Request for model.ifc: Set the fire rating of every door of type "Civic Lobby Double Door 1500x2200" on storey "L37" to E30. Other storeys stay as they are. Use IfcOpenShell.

First a look at what the model holds.

```python
import ifcopenshell
import ifcopenshell.util.element

model = ifcopenshell.open("model.ifc")
print(model.schema)
storey = next(s for s in model.by_type("IfcBuildingStorey") if s.Name == "L37")
doors = [e for e in ifcopenshell.util.element.get_decomposition(storey) if e.is_a("IfcDoor")]
seen = {}
for e in doors:
    element_type = ifcopenshell.util.element.get_type(e)
    key = (element_type.Name if element_type != e and element_type else None, ifcopenshell.util.element.get_pset(e, "Pset_DoorCommon", "FireRating"))
    seen[key] = seen.get(key, 0) + 1
for (name, value), count in sorted(seen.items(), key=str):
    print(count, "x", name, "|", value)
```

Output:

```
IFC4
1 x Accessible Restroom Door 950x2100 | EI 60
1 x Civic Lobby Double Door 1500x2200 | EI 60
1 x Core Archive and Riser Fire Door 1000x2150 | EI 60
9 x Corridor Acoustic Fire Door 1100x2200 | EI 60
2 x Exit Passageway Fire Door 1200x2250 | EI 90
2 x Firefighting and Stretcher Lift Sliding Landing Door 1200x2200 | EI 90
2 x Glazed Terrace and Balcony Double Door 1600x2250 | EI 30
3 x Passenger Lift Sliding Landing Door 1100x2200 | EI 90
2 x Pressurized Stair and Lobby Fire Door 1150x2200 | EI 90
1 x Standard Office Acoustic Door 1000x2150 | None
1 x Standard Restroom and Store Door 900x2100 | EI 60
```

```python
import ifcopenshell
import ifcopenshell.api.pset
import ifcopenshell.util.element

model = ifcopenshell.open("model.ifc")

storey = next(s for s in model.by_type("IfcBuildingStorey") if s.Name == "L37")
doors = [e for e in ifcopenshell.util.element.get_decomposition(storey) if e.is_a("IfcDoor")]

count = 0
for e in doors:
    element_type = ifcopenshell.util.element.get_type(e)
    if element_type in (None, e) or element_type.Name != "Civic Lobby Double Door 1500x2200":
        continue
    found = ifcopenshell.util.element.get_pset(e, "Pset_DoorCommon", should_inherit=False)
    if found:
        pset = model.by_id(found["id"])
        if len(ifcopenshell.util.element.get_elements_by_pset(pset)) > 1:
            pset = ifcopenshell.api.pset.unshare_pset(model, products=[e], pset=pset)[0]
    else:
        pset = ifcopenshell.api.pset.add_pset(model, product=e, name="Pset_DoorCommon")
    ifcopenshell.api.pset.edit_pset(model, pset=pset, properties={"FireRating": "E30"})
    count += 1

print(count, "doors updated")

model.write("model_edited.ifc")
```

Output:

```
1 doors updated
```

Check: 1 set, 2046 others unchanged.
